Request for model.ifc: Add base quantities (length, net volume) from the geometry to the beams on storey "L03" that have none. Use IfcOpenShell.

First a look at what the model holds.

```python
import ifcopenshell
import ifcopenshell.util.element
import ifcopenshell.util.unit

model = ifcopenshell.open("model.ifc")
print(model.schema)
for unit_type in ("LENGTHUNIT", "AREAUNIT", "VOLUMEUNIT"):
    print(unit_type, ifcopenshell.util.unit.calculate_unit_scale(model, unit_type))
storey = next(s for s in model.by_type("IfcBuildingStorey") if s.Name == "L03")
beams = [e for e in ifcopenshell.util.element.get_decomposition(storey) if e.is_a("IfcBeam")]
for e in sorted(beams, key=lambda e: e.id()):
    print(e.id(), e.is_a(), e.Name, list(ifcopenshell.util.element.get_psets(e, qtos_only=True)), sep=" | ")
```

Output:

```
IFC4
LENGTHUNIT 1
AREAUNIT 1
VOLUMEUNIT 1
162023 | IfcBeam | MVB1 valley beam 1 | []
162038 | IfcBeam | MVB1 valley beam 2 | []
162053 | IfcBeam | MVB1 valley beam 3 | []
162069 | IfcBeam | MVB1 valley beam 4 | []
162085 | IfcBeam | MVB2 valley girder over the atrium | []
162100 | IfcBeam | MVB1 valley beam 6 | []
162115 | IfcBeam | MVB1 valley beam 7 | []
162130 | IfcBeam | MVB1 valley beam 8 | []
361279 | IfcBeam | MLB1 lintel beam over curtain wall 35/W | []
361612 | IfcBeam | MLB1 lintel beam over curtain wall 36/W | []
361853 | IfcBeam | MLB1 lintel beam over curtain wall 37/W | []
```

```python
import ifcopenshell
import ifcopenshell.api.pset
import ifcopenshell.geom
import ifcopenshell.util.element
import ifcopenshell.util.shape
import ifcopenshell.util.unit

model = ifcopenshell.open("model.ifc")
unit_scale = ifcopenshell.util.unit.calculate_unit_scale(model)
volume_scale = ifcopenshell.util.unit.calculate_unit_scale(model, "VOLUMEUNIT")
settings = ifcopenshell.geom.settings()

storey = next(s for s in model.by_type("IfcBuildingStorey") if s.Name == "L03")
beams = [e for e in ifcopenshell.util.element.get_decomposition(storey) if e.is_a("IfcBeam")]

for e in sorted(beams, key=lambda e: e.id()):
    if ifcopenshell.util.element.get_psets(e, qtos_only=True, should_inherit=False):
        continue
    # Geometry comes back in metres, in the element's own axes.
    shape = ifcopenshell.geom.create_shape(settings, e)
    values = {
        "Length": ifcopenshell.util.shape.get_max_xyz(shape.geometry) / unit_scale,
        "NetVolume": ifcopenshell.util.shape.get_volume(shape.geometry) / volume_scale,
    }
    qto = ifcopenshell.api.pset.add_qto(model, product=e, name="Qto_BeamBaseQuantities")
    ifcopenshell.api.pset.edit_qto(model, qto=qto, properties=values)
    print(e.id(), {k: round(v, 3) for k, v in values.items()})

model.write("model_v2.ifc")
```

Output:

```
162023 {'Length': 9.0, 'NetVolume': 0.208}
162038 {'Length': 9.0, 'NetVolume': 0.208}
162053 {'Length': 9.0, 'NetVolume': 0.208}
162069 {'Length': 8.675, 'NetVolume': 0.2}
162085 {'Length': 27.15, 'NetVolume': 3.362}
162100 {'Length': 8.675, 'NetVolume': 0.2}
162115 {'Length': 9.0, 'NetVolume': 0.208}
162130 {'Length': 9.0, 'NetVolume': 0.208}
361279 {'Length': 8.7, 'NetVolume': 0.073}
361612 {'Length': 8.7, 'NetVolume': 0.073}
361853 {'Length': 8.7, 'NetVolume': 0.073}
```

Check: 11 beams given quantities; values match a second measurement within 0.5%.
